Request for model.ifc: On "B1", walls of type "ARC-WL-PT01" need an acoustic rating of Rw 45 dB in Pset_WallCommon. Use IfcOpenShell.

First a look at what the model holds.

```python
import ifcopenshell
import ifcopenshell.util.element

model = ifcopenshell.open("model.ifc")
print(model.schema)
storey = next(s for s in model.by_type("IfcBuildingStorey") if s.Name == "B1")
walls = [e for e in ifcopenshell.util.element.get_decomposition(storey) if e.is_a("IfcWall")]
seen = {}
for e in walls:
    element_type = ifcopenshell.util.element.get_type(e)
    key = (element_type.Name if element_type != e and element_type else None, ifcopenshell.util.element.get_pset(e, "Pset_WallCommon", "AcousticRating"))
    seen[key] = seen.get(key, 0) + 1
for (name, value), count in sorted(seen.items(), key=str):
    print(count, "x", name, "|", value)
```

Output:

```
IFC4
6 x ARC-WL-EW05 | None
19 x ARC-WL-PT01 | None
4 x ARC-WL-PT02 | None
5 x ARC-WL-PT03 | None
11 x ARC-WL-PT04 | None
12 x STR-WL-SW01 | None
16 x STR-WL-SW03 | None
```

```python
import ifcopenshell
import ifcopenshell.api.pset
import ifcopenshell.util.element

model = ifcopenshell.open("model.ifc")

storey = next(s for s in model.by_type("IfcBuildingStorey") if s.Name == "B1")
walls = [e for e in ifcopenshell.util.element.get_decomposition(storey) if e.is_a("IfcWall")]

count = 0
for e in walls:
    element_type = ifcopenshell.util.element.get_type(e)
    if element_type in (None, e) or element_type.Name != "ARC-WL-PT01":
        continue
    # add_pset returns the element's existing set when there is one.
    pset = ifcopenshell.api.pset.add_pset(model, product=e, name="Pset_WallCommon")
    ifcopenshell.api.pset.edit_pset(model, pset=pset, properties={"AcousticRating": "Rw 45 dB"})
    count += 1

print(count, "walls updated")

model.write("model_edited.ifc")
```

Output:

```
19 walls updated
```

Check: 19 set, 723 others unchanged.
